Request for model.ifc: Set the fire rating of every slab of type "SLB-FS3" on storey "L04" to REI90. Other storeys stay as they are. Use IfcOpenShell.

First a look at what the model holds.

```python
import ifcopenshell
import ifcopenshell.util.element

model = ifcopenshell.open("model.ifc")
print(model.schema)
storey = next(s for s in model.by_type("IfcBuildingStorey") if s.Name == "L04")
slabs = [e for e in ifcopenshell.util.element.get_decomposition(storey) if e.is_a("IfcSlab")]
seen = {}
for e in slabs:
    element_type = ifcopenshell.util.element.get_type(e)
    key = (element_type.Name if element_type != e and element_type else None, ifcopenshell.util.element.get_pset(e, "Pset_SlabCommon", "FireRating"))
    seen[key] = seen.get(key, 0) + 1
for (name, value), count in sorted(seen.items(), key=str):
    print(count, "x", name, "|", value)
```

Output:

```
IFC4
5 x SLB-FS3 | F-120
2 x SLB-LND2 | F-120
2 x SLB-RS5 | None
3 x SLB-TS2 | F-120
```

```python
import ifcopenshell
import ifcopenshell.api.pset
import ifcopenshell.util.element

model = ifcopenshell.open("model.ifc")

storey = next(s for s in model.by_type("IfcBuildingStorey") if s.Name == "L04")
slabs = [e for e in ifcopenshell.util.element.get_decomposition(storey) if e.is_a("IfcSlab")]

count = 0
for e in slabs:
    element_type = ifcopenshell.util.element.get_type(e)
    if element_type in (None, e) or element_type.Name != "SLB-FS3":
        continue
    # add_pset returns the element's existing set when there is one.
    pset = ifcopenshell.api.pset.add_pset(model, product=e, name="Pset_SlabCommon")
    ifcopenshell.api.pset.edit_pset(model, pset=pset, properties={"FireRating": "REI90"})
    count += 1

print(count, "slabs updated")

model.write("model_rev.ifc")
```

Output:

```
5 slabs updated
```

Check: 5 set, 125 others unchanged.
